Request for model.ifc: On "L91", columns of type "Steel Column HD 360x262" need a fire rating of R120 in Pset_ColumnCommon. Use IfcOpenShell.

First a look at what the model holds.

```python
import ifcopenshell
import ifcopenshell.util.element

model = ifcopenshell.open("model.ifc")
print(model.schema)
storey = next(s for s in model.by_type("IfcBuildingStorey") if s.Name == "L91")
columns = [e for e in ifcopenshell.util.element.get_decomposition(storey) if e.is_a("IfcColumn")]
seen = {}
for e in columns:
    element_type = ifcopenshell.util.element.get_type(e)
    key = (element_type.Name if element_type != e and element_type else None, ifcopenshell.util.element.get_pset(e, "Pset_ColumnCommon", "FireRating"))
    seen[key] = seen.get(key, 0) + 1
for (name, value), count in sorted(seen.items(), key=str):
    print(count, "x", name, "|", value)
```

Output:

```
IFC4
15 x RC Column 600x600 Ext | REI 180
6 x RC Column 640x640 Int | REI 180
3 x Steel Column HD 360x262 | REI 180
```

```python
import ifcopenshell
import ifcopenshell.api.pset
import ifcopenshell.util.element

model = ifcopenshell.open("model.ifc")

storey = next(s for s in model.by_type("IfcBuildingStorey") if s.Name == "L91")
columns = [e for e in ifcopenshell.util.element.get_decomposition(storey) if e.is_a("IfcColumn")]

count = 0
for e in columns:
    element_type = ifcopenshell.util.element.get_type(e)
    if element_type in (None, e) or element_type.Name != "Steel Column HD 360x262":
        continue
    # add_pset returns the element's existing set when there is one.
    pset = ifcopenshell.api.pset.add_pset(model, product=e, name="Pset_ColumnCommon")
    ifcopenshell.api.pset.edit_pset(model, pset=pset, properties={"FireRating": "R120"})
    count += 1

print(count, "columns updated")

model.write("model_updated.ifc")
```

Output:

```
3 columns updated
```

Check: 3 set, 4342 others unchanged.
